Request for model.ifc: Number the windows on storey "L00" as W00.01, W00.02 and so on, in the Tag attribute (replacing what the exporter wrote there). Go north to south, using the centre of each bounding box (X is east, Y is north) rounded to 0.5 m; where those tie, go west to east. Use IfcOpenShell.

First a look at what the model holds.

```python
import ifcopenshell
import ifcopenshell.util.element
import ifcopenshell.util.placement

model = ifcopenshell.open("model.ifc")
print(model.schema)
storey = next(s for s in model.by_type("IfcBuildingStorey") if s.Name == "L00")
windows = [e for e in ifcopenshell.util.element.get_decomposition(storey) if e.is_a("IfcWindow")]
for e in sorted(windows, key=lambda e: e.id()):
    origin = ifcopenshell.util.placement.get_local_placement(e.ObjectPlacement)[:3, 3]
    print(e.id(), e.Tag, e.Name, origin.round(2) + 0.0, sep=" | ")
```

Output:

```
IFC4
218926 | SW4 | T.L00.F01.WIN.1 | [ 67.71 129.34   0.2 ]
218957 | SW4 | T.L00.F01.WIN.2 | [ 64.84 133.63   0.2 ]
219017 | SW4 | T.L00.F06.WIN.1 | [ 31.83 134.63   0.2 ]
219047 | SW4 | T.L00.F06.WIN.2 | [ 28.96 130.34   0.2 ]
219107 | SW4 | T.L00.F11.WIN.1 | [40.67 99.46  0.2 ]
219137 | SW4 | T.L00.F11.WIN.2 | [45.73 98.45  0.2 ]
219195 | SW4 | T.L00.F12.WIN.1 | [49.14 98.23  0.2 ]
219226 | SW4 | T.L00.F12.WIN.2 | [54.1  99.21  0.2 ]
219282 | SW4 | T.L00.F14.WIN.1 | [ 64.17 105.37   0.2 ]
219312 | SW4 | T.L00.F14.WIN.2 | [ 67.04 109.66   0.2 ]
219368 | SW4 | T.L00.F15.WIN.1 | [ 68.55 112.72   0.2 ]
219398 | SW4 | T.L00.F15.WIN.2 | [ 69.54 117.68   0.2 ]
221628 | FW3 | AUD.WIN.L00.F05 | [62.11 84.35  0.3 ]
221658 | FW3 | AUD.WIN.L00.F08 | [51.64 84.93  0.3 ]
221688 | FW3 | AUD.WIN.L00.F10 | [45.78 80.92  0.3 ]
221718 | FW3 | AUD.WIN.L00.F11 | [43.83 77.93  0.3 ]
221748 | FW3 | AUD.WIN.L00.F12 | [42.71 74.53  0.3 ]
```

```python
import ifcopenshell
import ifcopenshell.geom
import ifcopenshell.util.element
import ifcopenshell.util.shape

model = ifcopenshell.open("model.ifc")
settings = ifcopenshell.geom.settings()
settings.set("use-world-coords", True)


def centre(element):
    shape = ifcopenshell.geom.create_shape(settings, element)
    return ifcopenshell.util.shape.get_bbox_centroid(shape.geometry)


storey = next(s for s in model.by_type("IfcBuildingStorey") if s.Name == "L00")
windows = [e for e in ifcopenshell.util.element.get_decomposition(storey) if e.is_a("IfcWindow")]

# Insertion points can sit at a corner or the storey origin, so sort by the geometry (in metres).
centres = {e: centre(e) for e in windows}
windows.sort(key=lambda e: (-round(centres[e][1] / 0.5), centres[e][0]))

for i, e in enumerate(windows, start=1):
    number = f"W00.{i:02d}"
    e.Tag = number
    print(e.id(), number)

model.write("model_rev.ifc")
```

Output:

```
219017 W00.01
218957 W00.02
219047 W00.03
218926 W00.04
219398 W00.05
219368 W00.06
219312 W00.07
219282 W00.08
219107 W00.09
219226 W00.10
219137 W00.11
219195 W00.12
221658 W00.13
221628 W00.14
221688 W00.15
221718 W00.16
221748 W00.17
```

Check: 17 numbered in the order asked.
